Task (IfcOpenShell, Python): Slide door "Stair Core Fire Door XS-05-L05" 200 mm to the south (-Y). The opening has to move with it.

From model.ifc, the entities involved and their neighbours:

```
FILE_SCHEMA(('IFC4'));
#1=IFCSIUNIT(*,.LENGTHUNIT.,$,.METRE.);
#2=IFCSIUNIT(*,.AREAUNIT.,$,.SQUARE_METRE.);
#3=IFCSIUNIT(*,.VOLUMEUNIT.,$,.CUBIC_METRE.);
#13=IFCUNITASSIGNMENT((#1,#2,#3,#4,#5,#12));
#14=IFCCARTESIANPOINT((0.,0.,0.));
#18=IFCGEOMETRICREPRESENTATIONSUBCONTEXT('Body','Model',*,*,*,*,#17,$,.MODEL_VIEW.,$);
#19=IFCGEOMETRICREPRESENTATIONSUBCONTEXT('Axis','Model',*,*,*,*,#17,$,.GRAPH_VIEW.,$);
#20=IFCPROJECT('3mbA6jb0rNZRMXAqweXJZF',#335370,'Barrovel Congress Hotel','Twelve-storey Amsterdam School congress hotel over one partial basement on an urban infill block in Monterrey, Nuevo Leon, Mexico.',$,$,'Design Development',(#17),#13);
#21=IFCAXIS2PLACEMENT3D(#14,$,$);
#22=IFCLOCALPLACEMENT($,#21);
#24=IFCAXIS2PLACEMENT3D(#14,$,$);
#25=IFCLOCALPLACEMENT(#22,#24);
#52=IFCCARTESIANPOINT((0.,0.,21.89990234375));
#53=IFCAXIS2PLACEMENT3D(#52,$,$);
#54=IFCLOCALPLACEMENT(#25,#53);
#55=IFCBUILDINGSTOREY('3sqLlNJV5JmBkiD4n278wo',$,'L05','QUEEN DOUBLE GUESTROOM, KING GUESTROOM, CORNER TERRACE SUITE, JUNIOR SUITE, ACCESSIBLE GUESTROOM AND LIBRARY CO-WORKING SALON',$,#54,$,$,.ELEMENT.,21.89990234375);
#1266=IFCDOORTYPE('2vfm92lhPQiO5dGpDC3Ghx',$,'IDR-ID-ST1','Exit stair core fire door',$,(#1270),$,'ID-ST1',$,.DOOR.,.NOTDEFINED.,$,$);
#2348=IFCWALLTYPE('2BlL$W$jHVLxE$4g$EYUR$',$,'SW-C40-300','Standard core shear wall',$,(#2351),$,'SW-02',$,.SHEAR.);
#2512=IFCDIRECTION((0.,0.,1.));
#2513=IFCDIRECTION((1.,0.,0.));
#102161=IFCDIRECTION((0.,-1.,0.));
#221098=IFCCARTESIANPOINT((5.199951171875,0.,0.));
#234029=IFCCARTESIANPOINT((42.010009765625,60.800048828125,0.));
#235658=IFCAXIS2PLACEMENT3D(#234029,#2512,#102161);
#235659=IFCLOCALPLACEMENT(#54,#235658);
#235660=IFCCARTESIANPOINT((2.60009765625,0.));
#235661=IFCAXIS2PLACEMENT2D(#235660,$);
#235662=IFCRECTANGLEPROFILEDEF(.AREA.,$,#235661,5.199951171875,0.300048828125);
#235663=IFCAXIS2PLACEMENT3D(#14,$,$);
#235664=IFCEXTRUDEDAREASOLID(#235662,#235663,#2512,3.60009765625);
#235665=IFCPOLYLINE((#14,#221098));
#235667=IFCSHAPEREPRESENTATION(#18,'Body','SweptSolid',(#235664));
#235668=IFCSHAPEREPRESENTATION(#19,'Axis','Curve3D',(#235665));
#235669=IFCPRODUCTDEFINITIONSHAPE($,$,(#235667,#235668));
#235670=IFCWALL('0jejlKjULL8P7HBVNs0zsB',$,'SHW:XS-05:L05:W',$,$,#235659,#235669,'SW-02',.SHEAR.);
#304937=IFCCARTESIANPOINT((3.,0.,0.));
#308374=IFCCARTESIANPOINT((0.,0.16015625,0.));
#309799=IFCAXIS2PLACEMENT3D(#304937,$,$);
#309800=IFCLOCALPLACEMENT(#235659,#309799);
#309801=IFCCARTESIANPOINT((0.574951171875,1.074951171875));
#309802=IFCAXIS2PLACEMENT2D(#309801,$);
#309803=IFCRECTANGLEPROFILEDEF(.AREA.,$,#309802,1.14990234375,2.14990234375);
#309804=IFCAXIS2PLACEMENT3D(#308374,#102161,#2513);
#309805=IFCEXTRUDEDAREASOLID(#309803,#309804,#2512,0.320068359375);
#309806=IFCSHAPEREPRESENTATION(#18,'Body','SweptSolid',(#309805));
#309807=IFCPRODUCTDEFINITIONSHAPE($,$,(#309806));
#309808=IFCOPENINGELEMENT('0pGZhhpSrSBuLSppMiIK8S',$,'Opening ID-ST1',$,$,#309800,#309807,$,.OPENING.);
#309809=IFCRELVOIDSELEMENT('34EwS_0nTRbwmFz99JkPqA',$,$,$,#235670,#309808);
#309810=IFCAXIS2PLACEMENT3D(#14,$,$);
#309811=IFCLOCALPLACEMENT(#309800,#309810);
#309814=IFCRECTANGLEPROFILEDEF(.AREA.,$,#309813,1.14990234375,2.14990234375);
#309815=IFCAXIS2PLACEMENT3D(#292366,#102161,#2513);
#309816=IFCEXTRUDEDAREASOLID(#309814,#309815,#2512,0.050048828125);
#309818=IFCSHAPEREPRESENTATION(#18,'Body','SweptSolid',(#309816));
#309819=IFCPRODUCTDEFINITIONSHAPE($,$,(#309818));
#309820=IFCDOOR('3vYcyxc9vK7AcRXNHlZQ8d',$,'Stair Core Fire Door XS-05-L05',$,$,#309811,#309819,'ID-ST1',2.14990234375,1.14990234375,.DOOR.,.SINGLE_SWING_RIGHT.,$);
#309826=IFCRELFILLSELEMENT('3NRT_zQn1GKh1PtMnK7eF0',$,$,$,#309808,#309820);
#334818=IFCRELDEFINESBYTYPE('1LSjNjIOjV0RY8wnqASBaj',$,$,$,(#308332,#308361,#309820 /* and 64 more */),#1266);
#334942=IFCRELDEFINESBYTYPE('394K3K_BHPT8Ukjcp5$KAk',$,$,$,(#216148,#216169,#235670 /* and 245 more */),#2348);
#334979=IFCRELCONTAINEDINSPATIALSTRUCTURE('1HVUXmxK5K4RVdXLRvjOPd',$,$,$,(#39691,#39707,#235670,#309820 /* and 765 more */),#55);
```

```python
import ifcopenshell
import ifcopenshell.api.geometry
import ifcopenshell.util.placement
import ifcopenshell.util.unit

model = ifcopenshell.open("model.ifc")
unit_scale = ifcopenshell.util.unit.calculate_unit_scale(model)

door = model.by_id(309820)
opening = door.FillsVoids[0].RelatingOpeningElement
wall = opening.VoidsElements[0].RelatingBuildingElement

wall_matrix = ifcopenshell.util.placement.get_local_placement(wall.ObjectPlacement)
shift = wall_matrix[:3, 0] * 0.2 / unit_scale
before = ifcopenshell.util.placement.get_local_placement(door.ObjectPlacement)[:3, 3].copy()

# The door is placed relative to its opening, so it follows when the opening moves.
matrix = ifcopenshell.util.placement.get_local_placement(opening.ObjectPlacement)
matrix[:3, 3] += shift
ifcopenshell.api.geometry.edit_object_placement(
    model, product=opening, matrix=matrix, is_si=False, should_transform_children=True
)

after = ifcopenshell.util.placement.get_local_placement(door.ObjectPlacement)[:3, 3]
print("door moved by", (after - before).round(3) + 0.0)

model.write("model-out.ifc")
```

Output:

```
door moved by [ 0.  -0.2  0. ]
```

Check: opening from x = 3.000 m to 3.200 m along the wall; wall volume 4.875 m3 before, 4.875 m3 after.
